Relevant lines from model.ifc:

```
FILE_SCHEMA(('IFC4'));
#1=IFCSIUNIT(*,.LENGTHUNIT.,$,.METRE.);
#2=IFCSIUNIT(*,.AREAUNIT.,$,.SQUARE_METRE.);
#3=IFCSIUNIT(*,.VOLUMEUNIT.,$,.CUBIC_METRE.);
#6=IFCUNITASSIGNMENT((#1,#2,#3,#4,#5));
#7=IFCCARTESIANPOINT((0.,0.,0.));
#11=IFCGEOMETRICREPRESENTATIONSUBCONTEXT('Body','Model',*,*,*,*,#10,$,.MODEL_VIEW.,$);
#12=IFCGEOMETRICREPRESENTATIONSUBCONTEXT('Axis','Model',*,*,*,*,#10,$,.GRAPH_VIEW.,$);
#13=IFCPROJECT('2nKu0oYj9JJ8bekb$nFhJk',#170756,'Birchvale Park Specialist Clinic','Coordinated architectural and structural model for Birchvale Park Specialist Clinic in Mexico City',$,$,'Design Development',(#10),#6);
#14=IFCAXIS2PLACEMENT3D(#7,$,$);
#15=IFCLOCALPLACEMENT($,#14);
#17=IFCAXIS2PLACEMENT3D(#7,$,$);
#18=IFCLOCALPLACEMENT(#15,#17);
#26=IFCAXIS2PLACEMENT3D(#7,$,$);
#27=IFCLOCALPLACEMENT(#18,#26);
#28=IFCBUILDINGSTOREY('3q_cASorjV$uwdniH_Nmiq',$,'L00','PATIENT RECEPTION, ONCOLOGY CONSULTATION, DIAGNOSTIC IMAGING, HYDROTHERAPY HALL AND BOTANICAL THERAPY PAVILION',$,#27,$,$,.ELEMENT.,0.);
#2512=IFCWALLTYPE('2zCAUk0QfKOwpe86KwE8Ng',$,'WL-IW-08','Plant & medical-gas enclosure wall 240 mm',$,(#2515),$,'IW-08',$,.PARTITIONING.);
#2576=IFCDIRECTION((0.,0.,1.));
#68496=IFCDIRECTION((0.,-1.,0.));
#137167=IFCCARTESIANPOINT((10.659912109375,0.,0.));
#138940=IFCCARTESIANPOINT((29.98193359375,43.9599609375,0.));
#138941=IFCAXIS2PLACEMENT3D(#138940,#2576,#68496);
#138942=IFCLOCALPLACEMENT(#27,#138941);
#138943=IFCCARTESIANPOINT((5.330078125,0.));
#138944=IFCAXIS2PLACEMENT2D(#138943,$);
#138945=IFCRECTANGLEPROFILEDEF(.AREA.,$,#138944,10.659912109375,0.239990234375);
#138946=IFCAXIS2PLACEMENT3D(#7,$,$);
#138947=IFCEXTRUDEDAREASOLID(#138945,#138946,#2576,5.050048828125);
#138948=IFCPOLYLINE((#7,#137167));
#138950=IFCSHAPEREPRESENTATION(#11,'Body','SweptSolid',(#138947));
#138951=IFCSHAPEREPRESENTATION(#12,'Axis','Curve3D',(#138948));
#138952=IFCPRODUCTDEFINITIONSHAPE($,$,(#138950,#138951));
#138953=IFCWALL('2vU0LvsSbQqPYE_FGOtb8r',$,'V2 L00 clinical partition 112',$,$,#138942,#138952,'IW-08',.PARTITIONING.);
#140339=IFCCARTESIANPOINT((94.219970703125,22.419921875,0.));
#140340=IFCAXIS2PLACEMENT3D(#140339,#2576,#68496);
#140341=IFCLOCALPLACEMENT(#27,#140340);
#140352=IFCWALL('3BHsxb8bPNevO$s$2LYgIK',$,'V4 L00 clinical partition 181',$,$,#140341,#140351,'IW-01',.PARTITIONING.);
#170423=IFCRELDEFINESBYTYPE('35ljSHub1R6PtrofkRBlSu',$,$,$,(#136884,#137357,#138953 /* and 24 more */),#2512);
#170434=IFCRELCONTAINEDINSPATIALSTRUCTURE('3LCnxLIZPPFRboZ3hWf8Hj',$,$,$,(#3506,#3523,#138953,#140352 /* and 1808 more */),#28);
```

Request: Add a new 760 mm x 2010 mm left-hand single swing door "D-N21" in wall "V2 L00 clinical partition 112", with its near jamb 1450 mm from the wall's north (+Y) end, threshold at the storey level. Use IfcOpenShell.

```python
import numpy as np
import ifcopenshell
import ifcopenshell.api.feature
import ifcopenshell.api.geometry
import ifcopenshell.api.root
import ifcopenshell.api.spatial
import ifcopenshell.geom
import ifcopenshell.util.element
import ifcopenshell.util.placement
import ifcopenshell.util.representation
import ifcopenshell.util.shape
import ifcopenshell.util.unit

model = ifcopenshell.open("model.ifc")
unit_scale = ifcopenshell.util.unit.calculate_unit_scale(model)
settings = ifcopenshell.geom.settings()


def volume(element):
    """Net volume in cubic metres, openings subtracted."""
    shape = ifcopenshell.geom.create_shape(settings, element)
    return ifcopenshell.util.shape.get_volume(shape.geometry)


wall = model.by_guid("2vU0LvsSbQqPYE_FGOtb8r")
storey = ifcopenshell.util.element.get_container(wall, ifc_class="IfcBuildingStorey")
context = ifcopenshell.util.representation.get_context(model, "Model", "Body", "MODEL_VIEW")
before = volume(wall)

width, height, from_end, sill = 0.76, 2.01, 1.45, 0.0  # metres

# The wall runs along its own X axis, and the end named is its -X end.
wall_shape = ifcopenshell.geom.create_shape(settings, wall)
x, y, z = ifcopenshell.util.shape.get_vertices(wall_shape.geometry).T
start = x.min() + from_end
face, thickness = float(y.min()), float(y.max() - y.min())
wall_matrix = ifcopenshell.util.placement.get_local_placement(wall.ObjectPlacement)
level = ifcopenshell.util.placement.get_local_placement(storey.ObjectPlacement)[2, 3]


def in_wall(x, y):
    """Placement at x, y metres in the wall's axes, at sill height."""
    matrix = wall_matrix.copy()
    matrix[:, 3] = wall_matrix @ np.array([x / unit_scale, y / unit_scale, 0.0, 1.0])
    matrix[2, 3] = level + sill / unit_scale
    return matrix


# Opening: a box that overshoots both wall faces by 50 mm.
opening = ifcopenshell.api.root.create_entity(model, ifc_class="IfcOpeningElement", predefined_type="OPENING")
box = ifcopenshell.api.geometry.add_wall_representation(
    model, context=context, length=width, height=height, thickness=thickness + 0.1
)
ifcopenshell.api.geometry.assign_representation(model, product=opening, representation=box)
ifcopenshell.api.geometry.edit_object_placement(model, product=opening, matrix=in_wall(start, face - 0.05), is_si=False)
ifcopenshell.api.feature.add_feature(model, feature=opening, element=wall)

door = ifcopenshell.api.root.create_entity(model, ifc_class="IfcDoor", name="D-N21", predefined_type="DOOR")
door.OverallWidth, door.OverallHeight = width / unit_scale, height / unit_scale
door.OperationType = "SINGLE_SWING_LEFT"
body = ifcopenshell.api.geometry.add_door_representation(
    model,
    context=context,
    overall_width=door.OverallWidth,
    overall_height=door.OverallHeight,
    operation_type="SINGLE_SWING_LEFT",
    lining_properties={"LiningDepth": thickness / unit_scale, "ThresholdDepth": thickness / unit_scale},
)
ifcopenshell.api.geometry.assign_representation(model, product=door, representation=body)
ifcopenshell.api.spatial.assign_container(model, products=[door], relating_structure=storey)
ifcopenshell.api.feature.add_filling(model, opening=opening, element=door)

# The lining spans the wall, so the door starts at the wall face.
ifcopenshell.api.geometry.edit_object_placement(model, product=door, matrix=in_wall(start, face), is_si=False)

after = volume(wall)

print(f"wall volume {before:.3f} -> {after:.3f} m3")

model.write("model-out.ifc")
```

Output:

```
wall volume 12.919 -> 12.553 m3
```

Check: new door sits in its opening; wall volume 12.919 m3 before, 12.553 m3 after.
